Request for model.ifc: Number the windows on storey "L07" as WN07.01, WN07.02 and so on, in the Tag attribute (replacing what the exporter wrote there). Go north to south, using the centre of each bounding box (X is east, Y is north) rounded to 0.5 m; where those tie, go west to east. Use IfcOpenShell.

First a look at what the model holds.

```python
import ifcopenshell
import ifcopenshell.util.element
import ifcopenshell.util.placement

model = ifcopenshell.open("model.ifc")
print(model.schema)
storey = next(s for s in model.by_type("IfcBuildingStorey") if s.Name == "L07")
windows = [e for e in ifcopenshell.util.element.get_decomposition(storey) if e.is_a("IfcWindow")]
for e in sorted(windows, key=lambda e: e.id()):
    origin = ifcopenshell.util.placement.get_local_placement(e.ObjectPlacement)[:3, 3]
    print(e.id(), e.Tag, e.Name, origin.round(2) + 0.0, sep=" | ")
```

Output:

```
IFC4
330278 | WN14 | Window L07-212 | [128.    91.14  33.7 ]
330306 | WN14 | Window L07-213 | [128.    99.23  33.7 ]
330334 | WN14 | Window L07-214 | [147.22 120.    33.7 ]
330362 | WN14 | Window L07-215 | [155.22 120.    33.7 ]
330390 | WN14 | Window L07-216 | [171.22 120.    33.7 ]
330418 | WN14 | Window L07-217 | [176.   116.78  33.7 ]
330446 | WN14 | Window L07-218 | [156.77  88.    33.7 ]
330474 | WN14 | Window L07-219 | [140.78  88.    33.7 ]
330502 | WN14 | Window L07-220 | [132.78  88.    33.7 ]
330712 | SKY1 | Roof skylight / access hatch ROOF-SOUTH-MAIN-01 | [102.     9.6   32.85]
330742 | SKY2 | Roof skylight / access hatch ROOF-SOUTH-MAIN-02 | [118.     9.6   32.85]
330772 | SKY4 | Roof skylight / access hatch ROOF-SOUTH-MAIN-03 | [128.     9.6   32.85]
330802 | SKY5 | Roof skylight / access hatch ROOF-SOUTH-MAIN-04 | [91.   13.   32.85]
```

```python
import ifcopenshell
import ifcopenshell.geom
import ifcopenshell.util.element
import ifcopenshell.util.shape

model = ifcopenshell.open("model.ifc")
settings = ifcopenshell.geom.settings()
settings.set("use-world-coords", True)


def centre(element):
    shape = ifcopenshell.geom.create_shape(settings, element)
    return ifcopenshell.util.shape.get_bbox_centroid(shape.geometry)


storey = next(s for s in model.by_type("IfcBuildingStorey") if s.Name == "L07")
windows = [e for e in ifcopenshell.util.element.get_decomposition(storey) if e.is_a("IfcWindow")]

# Insertion points can sit at a corner or the storey origin, so sort by the geometry (in metres).
centres = {e: centre(e) for e in windows}
windows.sort(key=lambda e: (-round(centres[e][1] / 0.5), centres[e][0]))

for i, e in enumerate(windows, start=1):
    number = f"WN07.{i:02d}"
    e.Tag = number
    print(e.id(), number)

model.write("model-out.ifc")
```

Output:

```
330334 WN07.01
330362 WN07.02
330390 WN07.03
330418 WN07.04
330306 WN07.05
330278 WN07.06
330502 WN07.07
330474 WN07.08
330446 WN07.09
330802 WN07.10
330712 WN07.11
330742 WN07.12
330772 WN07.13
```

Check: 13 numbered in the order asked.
